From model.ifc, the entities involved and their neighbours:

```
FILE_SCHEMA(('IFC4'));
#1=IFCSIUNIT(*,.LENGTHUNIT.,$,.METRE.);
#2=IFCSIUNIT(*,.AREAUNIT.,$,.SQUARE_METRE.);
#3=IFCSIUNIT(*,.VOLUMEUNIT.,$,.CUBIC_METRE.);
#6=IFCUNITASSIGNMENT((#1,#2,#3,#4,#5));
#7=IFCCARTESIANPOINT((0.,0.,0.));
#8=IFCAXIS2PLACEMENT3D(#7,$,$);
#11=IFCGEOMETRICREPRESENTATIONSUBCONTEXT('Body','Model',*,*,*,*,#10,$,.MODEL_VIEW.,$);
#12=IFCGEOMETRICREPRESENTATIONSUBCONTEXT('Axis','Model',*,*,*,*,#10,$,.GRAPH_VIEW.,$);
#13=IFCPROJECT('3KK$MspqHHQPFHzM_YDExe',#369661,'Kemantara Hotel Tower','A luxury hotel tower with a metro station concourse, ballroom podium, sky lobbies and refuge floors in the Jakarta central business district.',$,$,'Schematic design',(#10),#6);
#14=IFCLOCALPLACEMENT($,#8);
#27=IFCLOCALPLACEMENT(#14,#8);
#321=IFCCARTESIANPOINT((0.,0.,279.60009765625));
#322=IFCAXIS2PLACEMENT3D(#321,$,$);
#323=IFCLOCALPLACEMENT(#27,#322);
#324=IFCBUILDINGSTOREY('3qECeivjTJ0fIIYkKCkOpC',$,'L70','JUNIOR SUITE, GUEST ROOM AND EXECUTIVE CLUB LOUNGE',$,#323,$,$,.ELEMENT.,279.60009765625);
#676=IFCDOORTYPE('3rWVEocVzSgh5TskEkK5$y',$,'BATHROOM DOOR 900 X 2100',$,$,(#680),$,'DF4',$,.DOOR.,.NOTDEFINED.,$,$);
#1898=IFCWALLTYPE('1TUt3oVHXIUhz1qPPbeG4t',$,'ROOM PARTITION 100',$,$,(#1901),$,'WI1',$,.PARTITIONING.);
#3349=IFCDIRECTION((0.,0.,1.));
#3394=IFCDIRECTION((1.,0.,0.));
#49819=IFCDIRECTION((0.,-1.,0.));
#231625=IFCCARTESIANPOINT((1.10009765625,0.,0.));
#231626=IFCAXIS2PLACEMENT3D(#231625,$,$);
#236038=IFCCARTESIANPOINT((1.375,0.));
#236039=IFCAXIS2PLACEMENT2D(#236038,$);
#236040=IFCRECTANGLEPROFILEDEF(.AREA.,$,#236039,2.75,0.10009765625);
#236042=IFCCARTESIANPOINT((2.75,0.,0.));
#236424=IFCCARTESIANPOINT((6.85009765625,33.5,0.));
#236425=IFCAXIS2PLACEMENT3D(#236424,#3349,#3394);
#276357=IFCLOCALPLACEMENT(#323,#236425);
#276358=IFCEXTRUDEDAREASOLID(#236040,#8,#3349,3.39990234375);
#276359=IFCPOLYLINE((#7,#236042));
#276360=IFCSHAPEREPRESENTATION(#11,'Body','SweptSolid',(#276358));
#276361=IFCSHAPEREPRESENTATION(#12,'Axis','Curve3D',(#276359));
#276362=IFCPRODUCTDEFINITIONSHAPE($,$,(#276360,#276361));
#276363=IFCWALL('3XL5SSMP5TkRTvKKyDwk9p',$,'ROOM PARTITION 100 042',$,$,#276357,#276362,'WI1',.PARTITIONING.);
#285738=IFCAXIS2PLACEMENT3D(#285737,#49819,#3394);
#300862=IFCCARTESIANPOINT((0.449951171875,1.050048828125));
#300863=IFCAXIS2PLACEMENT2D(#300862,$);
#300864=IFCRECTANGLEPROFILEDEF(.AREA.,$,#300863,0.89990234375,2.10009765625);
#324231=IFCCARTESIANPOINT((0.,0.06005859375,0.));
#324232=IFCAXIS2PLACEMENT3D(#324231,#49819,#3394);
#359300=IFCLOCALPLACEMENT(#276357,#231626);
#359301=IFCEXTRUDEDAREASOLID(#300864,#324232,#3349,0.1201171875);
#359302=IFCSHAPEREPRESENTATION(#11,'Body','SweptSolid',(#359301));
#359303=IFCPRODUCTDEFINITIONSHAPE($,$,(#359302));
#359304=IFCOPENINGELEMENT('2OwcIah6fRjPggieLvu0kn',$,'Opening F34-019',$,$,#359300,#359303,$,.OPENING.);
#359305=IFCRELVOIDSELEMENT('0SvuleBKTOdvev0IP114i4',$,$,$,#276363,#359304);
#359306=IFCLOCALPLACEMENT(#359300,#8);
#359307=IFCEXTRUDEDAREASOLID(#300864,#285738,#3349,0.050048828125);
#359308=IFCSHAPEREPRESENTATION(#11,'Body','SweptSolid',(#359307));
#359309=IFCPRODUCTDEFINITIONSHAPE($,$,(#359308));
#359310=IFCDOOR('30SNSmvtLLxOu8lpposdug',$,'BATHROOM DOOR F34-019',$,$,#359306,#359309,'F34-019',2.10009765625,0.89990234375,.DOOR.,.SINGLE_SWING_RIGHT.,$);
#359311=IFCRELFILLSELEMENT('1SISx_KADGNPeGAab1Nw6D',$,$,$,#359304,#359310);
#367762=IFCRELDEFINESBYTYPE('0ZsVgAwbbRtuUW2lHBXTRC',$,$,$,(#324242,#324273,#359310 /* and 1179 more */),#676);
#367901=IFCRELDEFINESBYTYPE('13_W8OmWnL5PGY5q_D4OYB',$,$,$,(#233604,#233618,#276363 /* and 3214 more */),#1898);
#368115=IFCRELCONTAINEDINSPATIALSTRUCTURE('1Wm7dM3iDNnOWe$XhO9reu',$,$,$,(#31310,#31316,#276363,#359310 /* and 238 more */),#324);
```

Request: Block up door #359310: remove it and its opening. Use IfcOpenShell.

```python
import ifcopenshell
import ifcopenshell.api.feature
import ifcopenshell.api.root
import ifcopenshell.geom
import ifcopenshell.util.shape

model = ifcopenshell.open("model.ifc")
settings = ifcopenshell.geom.settings()


def volume(element):
    """Net volume in cubic metres, openings subtracted."""
    shape = ifcopenshell.geom.create_shape(settings, element)
    return ifcopenshell.util.shape.get_volume(shape.geometry)


door = model.by_guid("30SNSmvtLLxOu8lpposdug")
opening = door.FillsVoids[0].RelatingOpeningElement
wall = opening.VoidsElements[0].RelatingBuildingElement
before = volume(wall)

ifcopenshell.api.root.remove_product(model, product=door)
ifcopenshell.api.feature.remove_feature(model, feature=opening)

after = volume(wall)

print(f"wall volume {before:.3f} -> {after:.3f} m3")

model.write("model_v2.ifc")
```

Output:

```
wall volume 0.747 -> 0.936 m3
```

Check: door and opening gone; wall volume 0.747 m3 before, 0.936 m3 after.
